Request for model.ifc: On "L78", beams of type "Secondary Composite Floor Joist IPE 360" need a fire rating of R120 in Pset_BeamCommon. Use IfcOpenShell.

First a look at what the model holds.

```python
import ifcopenshell
import ifcopenshell.util.element

model = ifcopenshell.open("model.ifc")
print(model.schema)
storey = next(s for s in model.by_type("IfcBuildingStorey") if s.Name == "L78")
beams = [e for e in ifcopenshell.util.element.get_decomposition(storey) if e.is_a("IfcBeam")]
seen = {}
for e in beams:
    element_type = ifcopenshell.util.element.get_type(e)
    key = (element_type.Name if element_type != e and element_type else None, ifcopenshell.util.element.get_pset(e, "Pset_BeamCommon", "FireRating"))
    seen[key] = seen.get(key, 0) + 1
for (name, value), count in sorted(seen.items(), key=str):
    print(count, "x", name, "|", value)
```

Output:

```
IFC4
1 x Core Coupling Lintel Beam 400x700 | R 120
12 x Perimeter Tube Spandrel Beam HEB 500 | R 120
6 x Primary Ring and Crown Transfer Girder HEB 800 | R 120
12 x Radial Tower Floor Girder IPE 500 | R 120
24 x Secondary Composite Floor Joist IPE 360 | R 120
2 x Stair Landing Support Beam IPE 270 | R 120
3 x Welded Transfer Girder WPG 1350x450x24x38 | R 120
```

```python
import ifcopenshell
import ifcopenshell.api.pset
import ifcopenshell.util.element

model = ifcopenshell.open("model.ifc")

storey = next(s for s in model.by_type("IfcBuildingStorey") if s.Name == "L78")
beams = [e for e in ifcopenshell.util.element.get_decomposition(storey) if e.is_a("IfcBeam")]

count = 0
for e in beams:
    element_type = ifcopenshell.util.element.get_type(e)
    if element_type in (None, e) or element_type.Name != "Secondary Composite Floor Joist IPE 360":
        continue
    found = ifcopenshell.util.element.get_pset(e, "Pset_BeamCommon", should_inherit=False)
    if found:
        pset = model.by_id(found["id"])
        if len(ifcopenshell.util.element.get_elements_by_pset(pset)) > 1:
            pset = ifcopenshell.api.pset.unshare_pset(model, products=[e], pset=pset)[0]
    else:
        pset = ifcopenshell.api.pset.add_pset(model, product=e, name="Pset_BeamCommon")
    ifcopenshell.api.pset.edit_pset(model, pset=pset, properties={"FireRating": "R120"})
    count += 1

print(count, "beams updated")

model.write("model_v2.ifc")
```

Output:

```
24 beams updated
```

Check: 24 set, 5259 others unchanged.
